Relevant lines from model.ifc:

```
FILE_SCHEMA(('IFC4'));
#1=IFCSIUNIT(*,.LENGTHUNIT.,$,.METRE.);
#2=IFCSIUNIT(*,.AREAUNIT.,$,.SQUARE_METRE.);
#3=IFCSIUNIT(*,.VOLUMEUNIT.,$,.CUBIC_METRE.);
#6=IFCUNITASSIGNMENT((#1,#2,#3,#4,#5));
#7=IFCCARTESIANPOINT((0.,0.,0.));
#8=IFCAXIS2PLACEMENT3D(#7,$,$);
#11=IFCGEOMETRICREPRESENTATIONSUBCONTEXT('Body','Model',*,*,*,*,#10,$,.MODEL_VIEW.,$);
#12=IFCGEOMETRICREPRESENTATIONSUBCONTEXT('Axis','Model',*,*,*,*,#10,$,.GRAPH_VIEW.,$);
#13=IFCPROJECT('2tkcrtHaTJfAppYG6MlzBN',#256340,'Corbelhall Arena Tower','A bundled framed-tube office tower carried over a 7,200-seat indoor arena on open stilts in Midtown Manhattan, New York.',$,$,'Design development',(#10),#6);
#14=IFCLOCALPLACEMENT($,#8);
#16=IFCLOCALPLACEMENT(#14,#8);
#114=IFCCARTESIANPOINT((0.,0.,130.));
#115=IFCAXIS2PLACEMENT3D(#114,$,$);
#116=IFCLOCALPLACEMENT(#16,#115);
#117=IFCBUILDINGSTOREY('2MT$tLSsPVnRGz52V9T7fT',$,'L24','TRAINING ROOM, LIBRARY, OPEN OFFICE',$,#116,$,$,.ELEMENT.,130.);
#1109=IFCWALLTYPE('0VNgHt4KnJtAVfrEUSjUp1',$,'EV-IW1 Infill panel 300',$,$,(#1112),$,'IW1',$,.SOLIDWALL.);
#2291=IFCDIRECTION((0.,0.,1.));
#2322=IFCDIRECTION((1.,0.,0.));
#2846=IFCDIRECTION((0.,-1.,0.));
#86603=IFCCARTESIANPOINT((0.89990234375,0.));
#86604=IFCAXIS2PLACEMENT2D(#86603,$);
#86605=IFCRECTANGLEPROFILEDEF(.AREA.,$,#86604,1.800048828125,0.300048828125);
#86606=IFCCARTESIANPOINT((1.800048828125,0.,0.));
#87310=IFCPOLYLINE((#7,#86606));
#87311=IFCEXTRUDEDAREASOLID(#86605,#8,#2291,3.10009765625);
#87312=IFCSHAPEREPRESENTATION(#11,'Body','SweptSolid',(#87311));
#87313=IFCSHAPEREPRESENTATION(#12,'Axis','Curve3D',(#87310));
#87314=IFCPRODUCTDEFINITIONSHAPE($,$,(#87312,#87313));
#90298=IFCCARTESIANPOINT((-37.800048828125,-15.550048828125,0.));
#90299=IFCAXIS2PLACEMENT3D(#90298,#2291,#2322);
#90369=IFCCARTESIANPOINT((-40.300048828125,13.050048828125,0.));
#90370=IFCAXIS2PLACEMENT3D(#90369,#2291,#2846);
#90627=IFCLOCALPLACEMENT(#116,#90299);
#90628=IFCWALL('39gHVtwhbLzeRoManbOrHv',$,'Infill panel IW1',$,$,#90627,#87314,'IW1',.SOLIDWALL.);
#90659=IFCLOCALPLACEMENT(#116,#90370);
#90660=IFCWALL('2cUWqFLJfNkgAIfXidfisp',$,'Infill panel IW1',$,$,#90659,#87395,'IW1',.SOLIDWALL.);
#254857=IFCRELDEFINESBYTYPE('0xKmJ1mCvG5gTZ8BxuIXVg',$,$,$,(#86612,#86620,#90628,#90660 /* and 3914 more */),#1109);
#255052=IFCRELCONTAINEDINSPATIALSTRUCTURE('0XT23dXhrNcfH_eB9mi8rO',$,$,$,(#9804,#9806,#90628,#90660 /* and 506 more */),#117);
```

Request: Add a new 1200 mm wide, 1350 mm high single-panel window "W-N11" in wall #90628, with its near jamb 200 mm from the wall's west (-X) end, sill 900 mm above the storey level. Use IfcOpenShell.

```python
import numpy as np
import ifcopenshell
import ifcopenshell.api.feature
import ifcopenshell.api.geometry
import ifcopenshell.api.root
import ifcopenshell.api.spatial
import ifcopenshell.geom
import ifcopenshell.util.element
import ifcopenshell.util.placement
import ifcopenshell.util.representation
import ifcopenshell.util.shape
import ifcopenshell.util.unit

model = ifcopenshell.open("model.ifc")
unit_scale = ifcopenshell.util.unit.calculate_unit_scale(model)
settings = ifcopenshell.geom.settings()


def volume(element):
    """Net volume in cubic metres, openings subtracted."""
    shape = ifcopenshell.geom.create_shape(settings, element)
    return ifcopenshell.util.shape.get_volume(shape.geometry)


wall = model.by_guid("39gHVtwhbLzeRoManbOrHv")
storey = ifcopenshell.util.element.get_container(wall, ifc_class="IfcBuildingStorey")
context = ifcopenshell.util.representation.get_context(model, "Model", "Body", "MODEL_VIEW")
before = volume(wall)

width, height, from_end, sill = 1.2, 1.35, 0.2, 0.9  # metres

# The wall runs along its own X axis, and the end named is its -X end.
wall_shape = ifcopenshell.geom.create_shape(settings, wall)
x, y, z = ifcopenshell.util.shape.get_vertices(wall_shape.geometry).T
start = x.min() + from_end
face, thickness = float(y.min()), float(y.max() - y.min())
wall_matrix = ifcopenshell.util.placement.get_local_placement(wall.ObjectPlacement)
level = ifcopenshell.util.placement.get_local_placement(storey.ObjectPlacement)[2, 3]


def in_wall(x, y):
    """Placement at x, y metres in the wall's axes, at sill height."""
    matrix = wall_matrix.copy()
    matrix[:, 3] = wall_matrix @ np.array([x / unit_scale, y / unit_scale, 0.0, 1.0])
    matrix[2, 3] = level + sill / unit_scale
    return matrix


# Opening: a box that overshoots both wall faces by 50 mm.
opening = ifcopenshell.api.root.create_entity(model, ifc_class="IfcOpeningElement", predefined_type="OPENING")
box = ifcopenshell.api.geometry.add_wall_representation(
    model, context=context, length=width, height=height, thickness=thickness + 0.1
)
ifcopenshell.api.geometry.assign_representation(model, product=opening, representation=box)
ifcopenshell.api.geometry.edit_object_placement(model, product=opening, matrix=in_wall(start, face - 0.05), is_si=False)
ifcopenshell.api.feature.add_feature(model, feature=opening, element=wall)

window = ifcopenshell.api.root.create_entity(model, ifc_class="IfcWindow", name="W-N11", predefined_type="WINDOW")
window.OverallWidth, window.OverallHeight = width / unit_scale, height / unit_scale
window.PartitioningType = "SINGLE_PANEL"
body = ifcopenshell.api.geometry.add_window_representation(
    model,
    context=context,
    overall_width=window.OverallWidth,
    overall_height=window.OverallHeight,
    partition_type="SINGLE_PANEL",
)
ifcopenshell.api.geometry.assign_representation(model, product=window, representation=body)
ifcopenshell.api.spatial.assign_container(model, products=[window], relating_structure=storey)
ifcopenshell.api.feature.add_filling(model, opening=opening, element=window)

# Centre the window in the wall's thickness.
ifcopenshell.api.geometry.edit_object_placement(model, product=window, matrix=in_wall(start, face), is_si=False)
window_shape = ifcopenshell.geom.create_shape(settings, window)
depth = ifcopenshell.util.shape.get_vertices(window_shape.geometry)[:, 1]
offset = face + thickness / 2 - (depth.min() + depth.max()) / 2
ifcopenshell.api.geometry.edit_object_placement(model, product=window, matrix=in_wall(start, offset), is_si=False)

after = volume(wall)

print(f"wall volume {before:.3f} -> {after:.3f} m3")

model.write("model_rev.ifc")
```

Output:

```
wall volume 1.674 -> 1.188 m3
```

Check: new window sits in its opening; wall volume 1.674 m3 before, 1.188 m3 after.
